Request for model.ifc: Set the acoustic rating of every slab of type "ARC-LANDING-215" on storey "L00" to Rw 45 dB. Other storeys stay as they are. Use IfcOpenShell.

First a look at what the model holds.

```python
import ifcopenshell
import ifcopenshell.util.element

model = ifcopenshell.open("model.ifc")
print(model.schema)
storey = next(s for s in model.by_type("IfcBuildingStorey") if s.Name == "L00")
slabs = [e for e in ifcopenshell.util.element.get_decomposition(storey) if e.is_a("IfcSlab")]
seen = {}
for e in slabs:
    element_type = ifcopenshell.util.element.get_type(e)
    key = (element_type.Name if element_type != e and element_type else None, ifcopenshell.util.element.get_pset(e, "Pset_SlabCommon", "AcousticRating"))
    seen[key] = seen.get(key, 0) + 1
for (name, value), count in sorted(seen.items(), key=str):
    print(count, "x", name, "|", value)
```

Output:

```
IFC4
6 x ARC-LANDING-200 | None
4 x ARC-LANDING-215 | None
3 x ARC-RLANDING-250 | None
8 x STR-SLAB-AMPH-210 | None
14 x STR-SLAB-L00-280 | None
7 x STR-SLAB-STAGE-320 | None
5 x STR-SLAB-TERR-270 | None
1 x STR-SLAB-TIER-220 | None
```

```python
import ifcopenshell
import ifcopenshell.api.pset
import ifcopenshell.util.element

model = ifcopenshell.open("model.ifc")

storey = next(s for s in model.by_type("IfcBuildingStorey") if s.Name == "L00")
slabs = [e for e in ifcopenshell.util.element.get_decomposition(storey) if e.is_a("IfcSlab")]

count = 0
for e in slabs:
    element_type = ifcopenshell.util.element.get_type(e)
    if element_type in (None, e) or element_type.Name != "ARC-LANDING-215":
        continue
    # add_pset returns the element's existing set when there is one.
    pset = ifcopenshell.api.pset.add_pset(model, product=e, name="Pset_SlabCommon")
    ifcopenshell.api.pset.edit_pset(model, pset=pset, properties={"AcousticRating": "Rw 45 dB"})
    count += 1

print(count, "slabs updated")

model.write("model_edited.ifc")
```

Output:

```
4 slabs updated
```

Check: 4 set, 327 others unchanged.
